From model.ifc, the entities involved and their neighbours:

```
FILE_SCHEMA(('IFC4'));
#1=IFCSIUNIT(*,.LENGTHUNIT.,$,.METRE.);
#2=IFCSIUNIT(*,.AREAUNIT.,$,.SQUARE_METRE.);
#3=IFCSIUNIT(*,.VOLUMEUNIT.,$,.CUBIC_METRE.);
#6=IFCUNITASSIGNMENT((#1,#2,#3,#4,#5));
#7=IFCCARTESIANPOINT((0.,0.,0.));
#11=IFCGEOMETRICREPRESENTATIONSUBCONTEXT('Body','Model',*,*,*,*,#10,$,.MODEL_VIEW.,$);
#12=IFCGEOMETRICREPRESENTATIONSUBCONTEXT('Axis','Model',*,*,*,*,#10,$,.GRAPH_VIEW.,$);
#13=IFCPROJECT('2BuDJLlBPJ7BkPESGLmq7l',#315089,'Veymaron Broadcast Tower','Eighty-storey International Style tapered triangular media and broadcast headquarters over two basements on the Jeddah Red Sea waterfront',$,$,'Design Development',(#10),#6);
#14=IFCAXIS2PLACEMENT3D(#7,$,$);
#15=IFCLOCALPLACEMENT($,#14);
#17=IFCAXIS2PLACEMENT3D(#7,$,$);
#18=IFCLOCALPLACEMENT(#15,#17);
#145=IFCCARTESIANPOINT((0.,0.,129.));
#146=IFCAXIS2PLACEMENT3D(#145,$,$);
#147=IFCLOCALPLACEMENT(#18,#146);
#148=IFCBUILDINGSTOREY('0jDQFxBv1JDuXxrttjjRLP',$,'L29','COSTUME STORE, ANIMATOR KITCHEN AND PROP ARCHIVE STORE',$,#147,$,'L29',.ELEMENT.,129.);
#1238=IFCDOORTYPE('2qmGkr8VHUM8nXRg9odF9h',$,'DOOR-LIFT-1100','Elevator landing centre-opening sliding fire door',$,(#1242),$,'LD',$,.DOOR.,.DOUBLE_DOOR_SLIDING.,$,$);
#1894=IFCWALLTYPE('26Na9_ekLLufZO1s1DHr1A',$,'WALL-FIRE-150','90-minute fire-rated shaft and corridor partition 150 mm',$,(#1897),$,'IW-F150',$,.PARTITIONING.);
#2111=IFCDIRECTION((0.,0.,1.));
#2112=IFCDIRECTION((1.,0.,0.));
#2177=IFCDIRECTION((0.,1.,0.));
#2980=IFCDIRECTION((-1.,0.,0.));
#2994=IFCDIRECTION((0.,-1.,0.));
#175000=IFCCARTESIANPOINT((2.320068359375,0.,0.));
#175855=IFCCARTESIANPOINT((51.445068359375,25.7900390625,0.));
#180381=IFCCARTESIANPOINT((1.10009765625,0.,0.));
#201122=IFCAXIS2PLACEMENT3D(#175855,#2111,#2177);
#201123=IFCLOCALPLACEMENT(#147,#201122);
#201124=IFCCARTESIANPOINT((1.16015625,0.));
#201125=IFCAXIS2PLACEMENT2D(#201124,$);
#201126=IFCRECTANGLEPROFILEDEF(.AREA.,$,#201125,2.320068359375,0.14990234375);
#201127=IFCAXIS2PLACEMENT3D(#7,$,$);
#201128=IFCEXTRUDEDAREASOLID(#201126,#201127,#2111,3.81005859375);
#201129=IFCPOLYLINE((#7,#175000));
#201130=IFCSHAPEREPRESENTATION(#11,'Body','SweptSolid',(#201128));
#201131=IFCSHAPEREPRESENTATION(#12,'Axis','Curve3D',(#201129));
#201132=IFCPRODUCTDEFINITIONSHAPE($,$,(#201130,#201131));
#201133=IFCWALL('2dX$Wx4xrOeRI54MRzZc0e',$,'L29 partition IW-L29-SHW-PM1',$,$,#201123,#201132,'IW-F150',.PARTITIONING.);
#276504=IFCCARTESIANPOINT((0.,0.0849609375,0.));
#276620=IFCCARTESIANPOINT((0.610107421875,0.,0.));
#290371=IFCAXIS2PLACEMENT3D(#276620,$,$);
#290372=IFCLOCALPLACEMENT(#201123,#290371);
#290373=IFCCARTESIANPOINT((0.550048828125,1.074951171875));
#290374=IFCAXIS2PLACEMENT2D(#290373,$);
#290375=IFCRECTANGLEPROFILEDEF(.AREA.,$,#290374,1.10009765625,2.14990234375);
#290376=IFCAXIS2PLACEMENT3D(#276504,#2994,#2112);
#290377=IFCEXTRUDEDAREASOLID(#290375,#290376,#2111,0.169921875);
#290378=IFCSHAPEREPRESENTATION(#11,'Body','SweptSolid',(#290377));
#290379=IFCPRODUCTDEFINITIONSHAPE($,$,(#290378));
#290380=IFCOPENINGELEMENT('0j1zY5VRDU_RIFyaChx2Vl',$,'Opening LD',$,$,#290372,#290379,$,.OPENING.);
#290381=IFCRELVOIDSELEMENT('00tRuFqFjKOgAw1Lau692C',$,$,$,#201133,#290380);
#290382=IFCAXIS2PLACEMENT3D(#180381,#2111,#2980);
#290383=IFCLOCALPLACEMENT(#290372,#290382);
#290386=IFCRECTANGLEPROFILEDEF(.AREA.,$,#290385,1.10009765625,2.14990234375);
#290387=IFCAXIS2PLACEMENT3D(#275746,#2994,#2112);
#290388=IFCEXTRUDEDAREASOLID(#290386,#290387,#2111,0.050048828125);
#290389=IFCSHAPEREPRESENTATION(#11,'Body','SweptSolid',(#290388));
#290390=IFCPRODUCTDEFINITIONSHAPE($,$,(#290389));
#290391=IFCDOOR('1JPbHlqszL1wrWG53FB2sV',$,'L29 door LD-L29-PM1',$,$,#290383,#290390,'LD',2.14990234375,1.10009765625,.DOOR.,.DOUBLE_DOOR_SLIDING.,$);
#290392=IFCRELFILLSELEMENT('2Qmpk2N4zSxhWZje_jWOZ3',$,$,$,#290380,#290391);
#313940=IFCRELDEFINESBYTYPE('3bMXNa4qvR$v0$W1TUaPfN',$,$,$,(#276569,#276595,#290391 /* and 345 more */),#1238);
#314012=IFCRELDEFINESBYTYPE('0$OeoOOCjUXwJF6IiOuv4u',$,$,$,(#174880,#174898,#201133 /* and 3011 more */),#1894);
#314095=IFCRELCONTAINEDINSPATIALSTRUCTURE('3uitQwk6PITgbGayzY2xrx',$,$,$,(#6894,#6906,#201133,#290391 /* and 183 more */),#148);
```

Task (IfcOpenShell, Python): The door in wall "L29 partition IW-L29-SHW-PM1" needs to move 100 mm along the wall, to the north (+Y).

```python
import ifcopenshell
import ifcopenshell.api.geometry
import ifcopenshell.util.placement
import ifcopenshell.util.unit

model = ifcopenshell.open("model.ifc")
unit_scale = ifcopenshell.util.unit.calculate_unit_scale(model)

door = model.by_id(290391)
opening = door.FillsVoids[0].RelatingOpeningElement
wall = opening.VoidsElements[0].RelatingBuildingElement

wall_matrix = ifcopenshell.util.placement.get_local_placement(wall.ObjectPlacement)
shift = wall_matrix[:3, 0] * 0.1 / unit_scale
before = ifcopenshell.util.placement.get_local_placement(door.ObjectPlacement)[:3, 3].copy()

# The door is placed relative to its opening, so it follows when the opening moves.
matrix = ifcopenshell.util.placement.get_local_placement(opening.ObjectPlacement)
matrix[:3, 3] += shift
ifcopenshell.api.geometry.edit_object_placement(
    model, product=opening, matrix=matrix, is_si=False, should_transform_children=True
)

after = ifcopenshell.util.placement.get_local_placement(door.ObjectPlacement)[:3, 3]
print("door moved by", (after - before).round(3) + 0.0)

model.write("model_v2.ifc")
```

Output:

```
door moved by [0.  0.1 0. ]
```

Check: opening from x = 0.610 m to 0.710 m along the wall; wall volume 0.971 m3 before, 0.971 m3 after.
